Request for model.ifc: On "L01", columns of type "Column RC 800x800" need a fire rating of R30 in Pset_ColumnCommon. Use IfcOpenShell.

First a look at what the model holds.

```python
import ifcopenshell
import ifcopenshell.util.element

model = ifcopenshell.open("model.ifc")
print(model.schema)
storey = next(s for s in model.by_type("IfcBuildingStorey") if s.Name == "L01")
columns = [e for e in ifcopenshell.util.element.get_decomposition(storey) if e.is_a("IfcColumn")]
seen = {}
for e in columns:
    element_type = ifcopenshell.util.element.get_type(e)
    key = (element_type.Name if element_type != e and element_type else None, ifcopenshell.util.element.get_pset(e, "Pset_ColumnCommon", "FireRating"))
    seen[key] = seen.get(key, 0) + 1
for (name, value), count in sorted(seen.items(), key=str):
    print(count, "x", name, "|", value)
```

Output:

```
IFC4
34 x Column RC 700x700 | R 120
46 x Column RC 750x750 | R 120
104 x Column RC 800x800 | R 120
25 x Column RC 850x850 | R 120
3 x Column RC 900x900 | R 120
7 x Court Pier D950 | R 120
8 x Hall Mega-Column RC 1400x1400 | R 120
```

```python
import ifcopenshell
import ifcopenshell.api.pset
import ifcopenshell.util.element

model = ifcopenshell.open("model.ifc")

storey = next(s for s in model.by_type("IfcBuildingStorey") if s.Name == "L01")
columns = [e for e in ifcopenshell.util.element.get_decomposition(storey) if e.is_a("IfcColumn")]

count = 0
for e in columns:
    element_type = ifcopenshell.util.element.get_type(e)
    if element_type in (None, e) or element_type.Name != "Column RC 800x800":
        continue
    # add_pset returns the element's existing set when there is one.
    pset = ifcopenshell.api.pset.add_pset(model, product=e, name="Pset_ColumnCommon")
    ifcopenshell.api.pset.edit_pset(model, pset=pset, properties={"FireRating": "R30"})
    count += 1

print(count, "columns updated")

model.write("model_edited.ifc")
```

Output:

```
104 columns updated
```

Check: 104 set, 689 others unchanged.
